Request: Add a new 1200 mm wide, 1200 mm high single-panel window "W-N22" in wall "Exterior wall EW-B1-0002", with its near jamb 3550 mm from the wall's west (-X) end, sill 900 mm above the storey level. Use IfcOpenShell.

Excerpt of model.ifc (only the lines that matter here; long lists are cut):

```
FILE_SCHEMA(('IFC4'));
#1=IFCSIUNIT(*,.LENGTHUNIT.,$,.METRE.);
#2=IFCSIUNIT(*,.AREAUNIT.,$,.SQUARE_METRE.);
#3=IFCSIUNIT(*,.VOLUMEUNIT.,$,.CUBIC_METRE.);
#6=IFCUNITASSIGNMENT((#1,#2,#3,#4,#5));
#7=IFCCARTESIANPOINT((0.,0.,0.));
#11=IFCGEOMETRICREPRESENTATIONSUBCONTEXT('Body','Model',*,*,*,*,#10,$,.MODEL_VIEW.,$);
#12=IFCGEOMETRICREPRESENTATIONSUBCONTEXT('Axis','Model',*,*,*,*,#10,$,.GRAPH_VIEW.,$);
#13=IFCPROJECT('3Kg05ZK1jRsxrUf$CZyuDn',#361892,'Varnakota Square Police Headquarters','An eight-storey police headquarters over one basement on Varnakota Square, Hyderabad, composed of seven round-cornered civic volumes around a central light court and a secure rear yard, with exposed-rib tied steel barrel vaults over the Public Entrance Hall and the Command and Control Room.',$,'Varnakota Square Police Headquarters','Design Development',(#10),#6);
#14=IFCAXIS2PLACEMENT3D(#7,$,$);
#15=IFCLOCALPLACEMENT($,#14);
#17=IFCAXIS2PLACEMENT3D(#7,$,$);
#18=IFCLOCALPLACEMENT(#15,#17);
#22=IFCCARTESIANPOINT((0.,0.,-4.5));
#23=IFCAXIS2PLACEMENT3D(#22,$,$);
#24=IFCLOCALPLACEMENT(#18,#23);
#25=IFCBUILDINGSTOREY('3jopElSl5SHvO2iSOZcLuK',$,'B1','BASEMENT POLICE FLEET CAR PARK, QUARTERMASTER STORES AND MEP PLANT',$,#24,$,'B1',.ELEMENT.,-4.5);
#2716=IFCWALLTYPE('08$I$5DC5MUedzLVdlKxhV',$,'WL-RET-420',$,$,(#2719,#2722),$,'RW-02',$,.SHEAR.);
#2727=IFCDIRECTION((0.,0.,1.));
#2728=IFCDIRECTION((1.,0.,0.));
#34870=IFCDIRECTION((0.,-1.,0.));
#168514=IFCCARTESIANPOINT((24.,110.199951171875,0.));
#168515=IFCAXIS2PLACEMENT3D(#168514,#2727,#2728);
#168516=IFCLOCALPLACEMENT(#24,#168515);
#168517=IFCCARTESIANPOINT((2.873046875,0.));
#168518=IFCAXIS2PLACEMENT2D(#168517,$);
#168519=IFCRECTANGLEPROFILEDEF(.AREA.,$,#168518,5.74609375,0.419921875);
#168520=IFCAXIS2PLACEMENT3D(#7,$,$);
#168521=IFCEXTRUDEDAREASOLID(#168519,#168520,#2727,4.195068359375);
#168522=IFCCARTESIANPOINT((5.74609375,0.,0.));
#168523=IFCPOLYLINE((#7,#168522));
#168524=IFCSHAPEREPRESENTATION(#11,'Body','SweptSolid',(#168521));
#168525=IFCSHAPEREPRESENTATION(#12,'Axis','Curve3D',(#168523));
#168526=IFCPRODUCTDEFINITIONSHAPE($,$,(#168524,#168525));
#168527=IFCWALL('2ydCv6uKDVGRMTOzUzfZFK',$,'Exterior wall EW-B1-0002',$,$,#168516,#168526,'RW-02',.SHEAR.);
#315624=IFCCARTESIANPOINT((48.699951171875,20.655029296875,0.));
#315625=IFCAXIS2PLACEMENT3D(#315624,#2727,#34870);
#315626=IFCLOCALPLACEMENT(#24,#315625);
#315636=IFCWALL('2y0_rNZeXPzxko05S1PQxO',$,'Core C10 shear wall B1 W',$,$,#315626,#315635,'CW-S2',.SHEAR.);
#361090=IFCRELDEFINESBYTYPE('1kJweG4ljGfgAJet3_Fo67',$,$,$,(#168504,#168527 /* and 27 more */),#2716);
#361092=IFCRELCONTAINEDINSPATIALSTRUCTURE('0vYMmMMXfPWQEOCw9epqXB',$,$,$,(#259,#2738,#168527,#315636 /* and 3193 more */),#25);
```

```python
import numpy as np
import ifcopenshell
import ifcopenshell.api.feature
import ifcopenshell.api.geometry
import ifcopenshell.api.root
import ifcopenshell.api.spatial
import ifcopenshell.geom
import ifcopenshell.util.element
import ifcopenshell.util.placement
import ifcopenshell.util.representation
import ifcopenshell.util.shape
import ifcopenshell.util.unit

model = ifcopenshell.open("model.ifc")
unit_scale = ifcopenshell.util.unit.calculate_unit_scale(model)
settings = ifcopenshell.geom.settings()


def volume(element):
    """Net volume in cubic metres, openings subtracted."""
    shape = ifcopenshell.geom.create_shape(settings, element)
    return ifcopenshell.util.shape.get_volume(shape.geometry)


wall = model.by_guid("2ydCv6uKDVGRMTOzUzfZFK")
storey = ifcopenshell.util.element.get_container(wall, ifc_class="IfcBuildingStorey")
context = ifcopenshell.util.representation.get_context(model, "Model", "Body", "MODEL_VIEW")
before = volume(wall)

width, height, from_end, sill = 1.2, 1.2, 3.55, 0.9  # metres

# The wall runs along its own X axis, and the end named is its -X end.
wall_shape = ifcopenshell.geom.create_shape(settings, wall)
x, y, z = ifcopenshell.util.shape.get_vertices(wall_shape.geometry).T
start = x.min() + from_end
face, thickness = float(y.min()), float(y.max() - y.min())
wall_matrix = ifcopenshell.util.placement.get_local_placement(wall.ObjectPlacement)
level = ifcopenshell.util.placement.get_local_placement(storey.ObjectPlacement)[2, 3]


def in_wall(x, y):
    """Placement at x, y metres in the wall's axes, at sill height."""
    matrix = wall_matrix.copy()
    matrix[:, 3] = wall_matrix @ np.array([x / unit_scale, y / unit_scale, 0.0, 1.0])
    matrix[2, 3] = level + sill / unit_scale
    return matrix


# Opening: a box that overshoots both wall faces by 50 mm.
opening = ifcopenshell.api.root.create_entity(model, ifc_class="IfcOpeningElement", predefined_type="OPENING")
box = ifcopenshell.api.geometry.add_wall_representation(
    model, context=context, length=width, height=height, thickness=thickness + 0.1
)
ifcopenshell.api.geometry.assign_representation(model, product=opening, representation=box)
ifcopenshell.api.geometry.edit_object_placement(model, product=opening, matrix=in_wall(start, face - 0.05), is_si=False)
ifcopenshell.api.feature.add_feature(model, feature=opening, element=wall)

window = ifcopenshell.api.root.create_entity(model, ifc_class="IfcWindow", name="W-N22", predefined_type="WINDOW")
window.OverallWidth, window.OverallHeight = width / unit_scale, height / unit_scale
window.PartitioningType = "SINGLE_PANEL"
body = ifcopenshell.api.geometry.add_window_representation(
    model,
    context=context,
    overall_width=window.OverallWidth,
    overall_height=window.OverallHeight,
    partition_type="SINGLE_PANEL",
)
ifcopenshell.api.geometry.assign_representation(model, product=window, representation=body)
ifcopenshell.api.spatial.assign_container(model, products=[window], relating_structure=storey)
ifcopenshell.api.feature.add_filling(model, opening=opening, element=window)

# Centre the window in the wall's thickness.
ifcopenshell.api.geometry.edit_object_placement(model, product=window, matrix=in_wall(start, face), is_si=False)
window_shape = ifcopenshell.geom.create_shape(settings, window)
depth = ifcopenshell.util.shape.get_vertices(window_shape.geometry)[:, 1]
offset = face + thickness / 2 - (depth.min() + depth.max()) / 2
ifcopenshell.api.geometry.edit_object_placement(model, product=window, matrix=in_wall(start, offset), is_si=False)

after = volume(wall)

print(f"wall volume {before:.3f} -> {after:.3f} m3")

model.write("model_edited.ifc")
```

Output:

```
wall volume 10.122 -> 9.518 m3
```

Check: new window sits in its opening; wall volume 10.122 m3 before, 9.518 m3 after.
